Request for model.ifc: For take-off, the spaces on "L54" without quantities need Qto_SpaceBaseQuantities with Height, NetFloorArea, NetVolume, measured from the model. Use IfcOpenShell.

First a look at what the model holds.

```python
import ifcopenshell
import ifcopenshell.util.element
import ifcopenshell.util.unit

model = ifcopenshell.open("model.ifc")
print(model.schema)
for unit_type in ("LENGTHUNIT", "AREAUNIT", "VOLUMEUNIT"):
    print(unit_type, ifcopenshell.util.unit.calculate_unit_scale(model, unit_type))
storey = next(s for s in model.by_type("IfcBuildingStorey") if s.Name == "L54")
spaces = [e for e in ifcopenshell.util.element.get_decomposition(storey) if e.is_a("IfcSpace")]
for e in sorted(spaces, key=lambda e: e.id()):
    print(e.id(), e.is_a(), e.Name, list(ifcopenshell.util.element.get_psets(e, qtos_only=True)), sep=" | ")
```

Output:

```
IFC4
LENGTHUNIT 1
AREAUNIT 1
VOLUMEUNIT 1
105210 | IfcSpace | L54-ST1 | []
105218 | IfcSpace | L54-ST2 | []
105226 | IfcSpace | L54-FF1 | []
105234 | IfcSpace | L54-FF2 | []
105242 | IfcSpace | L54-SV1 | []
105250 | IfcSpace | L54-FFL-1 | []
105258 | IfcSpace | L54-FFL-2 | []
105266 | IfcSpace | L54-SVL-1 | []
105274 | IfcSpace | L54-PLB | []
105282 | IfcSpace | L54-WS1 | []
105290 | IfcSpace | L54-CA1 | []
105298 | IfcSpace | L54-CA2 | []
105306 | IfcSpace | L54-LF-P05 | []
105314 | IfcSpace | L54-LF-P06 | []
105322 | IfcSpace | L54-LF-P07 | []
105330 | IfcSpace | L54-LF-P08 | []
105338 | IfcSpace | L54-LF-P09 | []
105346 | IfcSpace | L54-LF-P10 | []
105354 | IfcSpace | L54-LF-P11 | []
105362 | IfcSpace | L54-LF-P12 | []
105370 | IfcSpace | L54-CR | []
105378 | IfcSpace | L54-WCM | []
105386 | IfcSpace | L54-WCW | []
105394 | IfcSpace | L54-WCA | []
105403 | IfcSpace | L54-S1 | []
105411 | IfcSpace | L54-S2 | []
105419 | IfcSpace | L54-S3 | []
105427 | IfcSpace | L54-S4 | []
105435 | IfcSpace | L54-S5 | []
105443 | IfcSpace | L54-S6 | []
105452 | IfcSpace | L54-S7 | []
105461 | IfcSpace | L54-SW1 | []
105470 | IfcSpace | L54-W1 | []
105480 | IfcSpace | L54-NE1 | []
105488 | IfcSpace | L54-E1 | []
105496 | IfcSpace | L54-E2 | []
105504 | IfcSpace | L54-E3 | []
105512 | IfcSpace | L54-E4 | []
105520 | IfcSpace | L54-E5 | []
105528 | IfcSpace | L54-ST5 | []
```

```python
import ifcopenshell
import ifcopenshell.api.pset
import ifcopenshell.geom
import ifcopenshell.util.element
import ifcopenshell.util.shape
import ifcopenshell.util.unit

model = ifcopenshell.open("model.ifc")
unit_scale = ifcopenshell.util.unit.calculate_unit_scale(model)
area_scale = ifcopenshell.util.unit.calculate_unit_scale(model, "AREAUNIT")
volume_scale = ifcopenshell.util.unit.calculate_unit_scale(model, "VOLUMEUNIT")
settings = ifcopenshell.geom.settings()

storey = next(s for s in model.by_type("IfcBuildingStorey") if s.Name == "L54")
spaces = [e for e in ifcopenshell.util.element.get_decomposition(storey) if e.is_a("IfcSpace")]

for e in sorted(spaces, key=lambda e: e.id()):
    if ifcopenshell.util.element.get_psets(e, qtos_only=True, should_inherit=False):
        continue
    # Geometry comes back in metres, in the element's own axes.
    shape = ifcopenshell.geom.create_shape(settings, e)
    values = {
        "Height": ifcopenshell.util.shape.get_z(shape.geometry) / unit_scale,
        "NetFloorArea": ifcopenshell.util.shape.get_footprint_area(shape.geometry) / area_scale,
        "NetVolume": ifcopenshell.util.shape.get_volume(shape.geometry) / volume_scale,
    }
    qto = ifcopenshell.api.pset.add_qto(model, product=e, name="Qto_SpaceBaseQuantities")
    ifcopenshell.api.pset.edit_qto(model, qto=qto, properties=values)
    print(e.id(), {k: round(v, 3) for k, v in values.items()})

model.write("model_edited.ifc")
```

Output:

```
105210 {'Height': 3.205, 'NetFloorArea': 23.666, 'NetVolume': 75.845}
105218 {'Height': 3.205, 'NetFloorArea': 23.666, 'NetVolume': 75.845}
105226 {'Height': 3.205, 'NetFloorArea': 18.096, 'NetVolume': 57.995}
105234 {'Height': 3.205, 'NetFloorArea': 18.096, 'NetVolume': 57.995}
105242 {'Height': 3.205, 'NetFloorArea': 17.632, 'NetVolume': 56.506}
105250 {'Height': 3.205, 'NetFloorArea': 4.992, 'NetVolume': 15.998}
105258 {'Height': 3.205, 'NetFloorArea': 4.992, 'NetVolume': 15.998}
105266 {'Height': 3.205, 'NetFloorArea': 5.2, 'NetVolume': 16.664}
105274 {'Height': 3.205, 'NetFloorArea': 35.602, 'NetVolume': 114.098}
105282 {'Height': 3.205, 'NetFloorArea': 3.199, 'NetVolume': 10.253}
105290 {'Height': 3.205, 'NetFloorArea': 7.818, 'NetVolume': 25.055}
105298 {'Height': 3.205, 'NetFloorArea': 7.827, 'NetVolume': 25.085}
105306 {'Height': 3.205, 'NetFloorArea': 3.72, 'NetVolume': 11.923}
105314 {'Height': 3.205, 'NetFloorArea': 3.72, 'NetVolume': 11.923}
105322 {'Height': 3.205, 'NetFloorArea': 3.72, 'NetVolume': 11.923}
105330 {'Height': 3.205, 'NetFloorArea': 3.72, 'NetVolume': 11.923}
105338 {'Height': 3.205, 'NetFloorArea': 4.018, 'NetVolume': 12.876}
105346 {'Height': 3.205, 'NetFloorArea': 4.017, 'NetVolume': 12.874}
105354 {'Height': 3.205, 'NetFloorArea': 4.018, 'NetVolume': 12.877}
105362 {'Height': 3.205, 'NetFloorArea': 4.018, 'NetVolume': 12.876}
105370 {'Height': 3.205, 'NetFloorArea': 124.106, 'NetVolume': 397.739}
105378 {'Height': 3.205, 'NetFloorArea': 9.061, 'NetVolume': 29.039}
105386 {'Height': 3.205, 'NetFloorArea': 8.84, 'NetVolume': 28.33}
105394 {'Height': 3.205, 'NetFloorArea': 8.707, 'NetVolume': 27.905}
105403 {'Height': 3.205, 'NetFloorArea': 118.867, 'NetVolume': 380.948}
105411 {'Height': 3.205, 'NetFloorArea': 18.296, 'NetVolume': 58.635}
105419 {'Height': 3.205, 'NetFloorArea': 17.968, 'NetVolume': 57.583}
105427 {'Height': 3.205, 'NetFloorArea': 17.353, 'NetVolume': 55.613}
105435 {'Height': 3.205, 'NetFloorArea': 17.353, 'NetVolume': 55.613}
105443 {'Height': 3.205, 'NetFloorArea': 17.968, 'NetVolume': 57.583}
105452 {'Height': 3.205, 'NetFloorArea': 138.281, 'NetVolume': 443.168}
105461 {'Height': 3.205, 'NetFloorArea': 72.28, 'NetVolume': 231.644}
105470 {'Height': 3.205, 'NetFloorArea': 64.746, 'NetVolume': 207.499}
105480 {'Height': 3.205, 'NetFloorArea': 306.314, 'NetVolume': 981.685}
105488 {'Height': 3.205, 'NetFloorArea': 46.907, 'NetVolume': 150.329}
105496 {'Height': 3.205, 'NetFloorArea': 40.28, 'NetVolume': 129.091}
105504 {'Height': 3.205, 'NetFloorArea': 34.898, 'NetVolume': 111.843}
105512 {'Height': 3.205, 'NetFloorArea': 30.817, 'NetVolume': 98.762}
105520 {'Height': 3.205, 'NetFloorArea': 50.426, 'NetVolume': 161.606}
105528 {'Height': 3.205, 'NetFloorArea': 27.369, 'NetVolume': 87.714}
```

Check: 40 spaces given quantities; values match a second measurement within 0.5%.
